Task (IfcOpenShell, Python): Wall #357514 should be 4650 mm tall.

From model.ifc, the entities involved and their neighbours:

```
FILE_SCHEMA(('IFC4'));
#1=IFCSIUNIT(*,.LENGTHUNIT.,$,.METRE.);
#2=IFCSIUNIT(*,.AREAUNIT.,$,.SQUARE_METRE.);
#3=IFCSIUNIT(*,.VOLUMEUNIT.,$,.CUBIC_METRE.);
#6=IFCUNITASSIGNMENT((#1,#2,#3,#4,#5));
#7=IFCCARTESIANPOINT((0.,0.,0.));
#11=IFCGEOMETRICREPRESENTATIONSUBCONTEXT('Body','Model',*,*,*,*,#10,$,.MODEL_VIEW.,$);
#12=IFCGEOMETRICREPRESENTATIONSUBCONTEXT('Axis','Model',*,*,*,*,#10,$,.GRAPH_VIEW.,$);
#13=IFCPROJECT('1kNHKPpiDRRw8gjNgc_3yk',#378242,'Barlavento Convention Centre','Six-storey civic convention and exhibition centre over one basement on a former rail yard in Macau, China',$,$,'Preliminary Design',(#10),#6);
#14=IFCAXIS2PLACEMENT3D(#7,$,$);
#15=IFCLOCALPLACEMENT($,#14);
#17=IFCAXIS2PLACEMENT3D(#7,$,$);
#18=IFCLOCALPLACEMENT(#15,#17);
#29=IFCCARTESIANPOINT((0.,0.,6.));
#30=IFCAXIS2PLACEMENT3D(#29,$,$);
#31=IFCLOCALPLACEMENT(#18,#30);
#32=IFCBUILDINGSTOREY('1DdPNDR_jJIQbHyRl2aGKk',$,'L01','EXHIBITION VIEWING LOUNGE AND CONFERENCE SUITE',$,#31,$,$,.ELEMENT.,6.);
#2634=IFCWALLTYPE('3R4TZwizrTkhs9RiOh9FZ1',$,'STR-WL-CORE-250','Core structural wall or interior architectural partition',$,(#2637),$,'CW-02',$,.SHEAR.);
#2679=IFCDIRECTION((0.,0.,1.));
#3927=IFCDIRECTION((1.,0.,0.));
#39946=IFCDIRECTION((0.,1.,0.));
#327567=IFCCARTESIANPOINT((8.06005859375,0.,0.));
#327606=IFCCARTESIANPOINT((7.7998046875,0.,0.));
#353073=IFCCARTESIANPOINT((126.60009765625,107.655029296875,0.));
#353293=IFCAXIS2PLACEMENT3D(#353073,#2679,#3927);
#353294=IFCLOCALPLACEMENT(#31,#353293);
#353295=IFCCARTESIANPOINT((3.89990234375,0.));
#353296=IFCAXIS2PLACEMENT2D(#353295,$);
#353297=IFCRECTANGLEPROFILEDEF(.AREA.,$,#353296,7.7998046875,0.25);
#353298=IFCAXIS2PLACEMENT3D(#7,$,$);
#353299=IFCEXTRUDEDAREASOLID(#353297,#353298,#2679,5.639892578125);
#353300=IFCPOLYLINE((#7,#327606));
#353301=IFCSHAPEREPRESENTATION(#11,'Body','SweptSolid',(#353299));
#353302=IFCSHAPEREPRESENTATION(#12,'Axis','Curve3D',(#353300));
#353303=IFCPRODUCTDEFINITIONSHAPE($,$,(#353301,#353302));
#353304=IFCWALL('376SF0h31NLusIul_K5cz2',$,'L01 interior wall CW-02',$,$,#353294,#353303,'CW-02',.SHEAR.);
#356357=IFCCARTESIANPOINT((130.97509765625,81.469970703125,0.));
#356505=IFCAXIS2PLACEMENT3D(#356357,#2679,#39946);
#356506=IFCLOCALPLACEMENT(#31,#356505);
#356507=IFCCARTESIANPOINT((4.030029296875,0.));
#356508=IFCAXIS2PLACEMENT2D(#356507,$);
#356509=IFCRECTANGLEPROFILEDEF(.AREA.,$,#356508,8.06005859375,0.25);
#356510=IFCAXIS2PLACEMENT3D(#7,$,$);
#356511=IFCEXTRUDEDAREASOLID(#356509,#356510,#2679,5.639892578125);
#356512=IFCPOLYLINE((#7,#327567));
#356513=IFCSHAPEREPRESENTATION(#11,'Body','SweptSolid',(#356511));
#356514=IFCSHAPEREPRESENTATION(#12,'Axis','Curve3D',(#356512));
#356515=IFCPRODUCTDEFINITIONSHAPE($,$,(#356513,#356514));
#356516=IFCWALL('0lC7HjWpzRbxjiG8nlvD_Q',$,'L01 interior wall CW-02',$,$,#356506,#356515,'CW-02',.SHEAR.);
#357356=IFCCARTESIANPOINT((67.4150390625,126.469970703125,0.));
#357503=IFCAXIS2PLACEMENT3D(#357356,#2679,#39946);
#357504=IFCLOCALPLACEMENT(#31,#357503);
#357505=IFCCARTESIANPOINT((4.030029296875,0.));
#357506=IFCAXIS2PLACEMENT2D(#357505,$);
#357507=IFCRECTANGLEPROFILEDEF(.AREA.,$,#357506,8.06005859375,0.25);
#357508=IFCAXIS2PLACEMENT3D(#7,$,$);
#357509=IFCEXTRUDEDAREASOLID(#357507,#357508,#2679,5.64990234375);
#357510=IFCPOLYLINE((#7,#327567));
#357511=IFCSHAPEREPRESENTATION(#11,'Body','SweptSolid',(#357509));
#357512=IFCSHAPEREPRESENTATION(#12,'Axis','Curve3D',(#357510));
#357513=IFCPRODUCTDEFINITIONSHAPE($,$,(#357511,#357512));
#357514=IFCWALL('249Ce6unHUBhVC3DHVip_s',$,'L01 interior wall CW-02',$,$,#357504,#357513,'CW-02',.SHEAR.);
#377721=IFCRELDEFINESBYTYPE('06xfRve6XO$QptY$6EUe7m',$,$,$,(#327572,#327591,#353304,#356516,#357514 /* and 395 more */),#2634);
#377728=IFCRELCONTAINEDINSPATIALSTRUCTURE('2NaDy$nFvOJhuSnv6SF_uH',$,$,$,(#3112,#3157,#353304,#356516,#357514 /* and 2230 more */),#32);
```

```python
import ifcopenshell
import ifcopenshell.geom
import ifcopenshell.util.representation
import ifcopenshell.util.shape
import ifcopenshell.util.unit

model = ifcopenshell.open("model.ifc")
unit_scale = ifcopenshell.util.unit.calculate_unit_scale(model)
settings = ifcopenshell.geom.settings()


def volume(element):
    """Net volume in cubic metres, openings subtracted."""
    shape = ifcopenshell.geom.create_shape(settings, element)
    return ifcopenshell.util.shape.get_volume(shape.geometry)


wall = model.by_guid("249Ce6unHUBhVC3DHVip_s")
before = volume(wall)

body = ifcopenshell.util.representation.get_representation(wall, "Model", "Body")
solid = body.Items[0]
old_height = solid.Depth
solid.Depth = 4.65 / unit_scale
after = volume(wall)

print(f"height {old_height:g} -> {solid.Depth:g}, volume {before:.3f} -> {after:.3f} m3")

model.write("model_updated.ifc")
```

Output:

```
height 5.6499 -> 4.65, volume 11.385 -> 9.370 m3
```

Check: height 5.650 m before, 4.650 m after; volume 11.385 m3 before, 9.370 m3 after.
